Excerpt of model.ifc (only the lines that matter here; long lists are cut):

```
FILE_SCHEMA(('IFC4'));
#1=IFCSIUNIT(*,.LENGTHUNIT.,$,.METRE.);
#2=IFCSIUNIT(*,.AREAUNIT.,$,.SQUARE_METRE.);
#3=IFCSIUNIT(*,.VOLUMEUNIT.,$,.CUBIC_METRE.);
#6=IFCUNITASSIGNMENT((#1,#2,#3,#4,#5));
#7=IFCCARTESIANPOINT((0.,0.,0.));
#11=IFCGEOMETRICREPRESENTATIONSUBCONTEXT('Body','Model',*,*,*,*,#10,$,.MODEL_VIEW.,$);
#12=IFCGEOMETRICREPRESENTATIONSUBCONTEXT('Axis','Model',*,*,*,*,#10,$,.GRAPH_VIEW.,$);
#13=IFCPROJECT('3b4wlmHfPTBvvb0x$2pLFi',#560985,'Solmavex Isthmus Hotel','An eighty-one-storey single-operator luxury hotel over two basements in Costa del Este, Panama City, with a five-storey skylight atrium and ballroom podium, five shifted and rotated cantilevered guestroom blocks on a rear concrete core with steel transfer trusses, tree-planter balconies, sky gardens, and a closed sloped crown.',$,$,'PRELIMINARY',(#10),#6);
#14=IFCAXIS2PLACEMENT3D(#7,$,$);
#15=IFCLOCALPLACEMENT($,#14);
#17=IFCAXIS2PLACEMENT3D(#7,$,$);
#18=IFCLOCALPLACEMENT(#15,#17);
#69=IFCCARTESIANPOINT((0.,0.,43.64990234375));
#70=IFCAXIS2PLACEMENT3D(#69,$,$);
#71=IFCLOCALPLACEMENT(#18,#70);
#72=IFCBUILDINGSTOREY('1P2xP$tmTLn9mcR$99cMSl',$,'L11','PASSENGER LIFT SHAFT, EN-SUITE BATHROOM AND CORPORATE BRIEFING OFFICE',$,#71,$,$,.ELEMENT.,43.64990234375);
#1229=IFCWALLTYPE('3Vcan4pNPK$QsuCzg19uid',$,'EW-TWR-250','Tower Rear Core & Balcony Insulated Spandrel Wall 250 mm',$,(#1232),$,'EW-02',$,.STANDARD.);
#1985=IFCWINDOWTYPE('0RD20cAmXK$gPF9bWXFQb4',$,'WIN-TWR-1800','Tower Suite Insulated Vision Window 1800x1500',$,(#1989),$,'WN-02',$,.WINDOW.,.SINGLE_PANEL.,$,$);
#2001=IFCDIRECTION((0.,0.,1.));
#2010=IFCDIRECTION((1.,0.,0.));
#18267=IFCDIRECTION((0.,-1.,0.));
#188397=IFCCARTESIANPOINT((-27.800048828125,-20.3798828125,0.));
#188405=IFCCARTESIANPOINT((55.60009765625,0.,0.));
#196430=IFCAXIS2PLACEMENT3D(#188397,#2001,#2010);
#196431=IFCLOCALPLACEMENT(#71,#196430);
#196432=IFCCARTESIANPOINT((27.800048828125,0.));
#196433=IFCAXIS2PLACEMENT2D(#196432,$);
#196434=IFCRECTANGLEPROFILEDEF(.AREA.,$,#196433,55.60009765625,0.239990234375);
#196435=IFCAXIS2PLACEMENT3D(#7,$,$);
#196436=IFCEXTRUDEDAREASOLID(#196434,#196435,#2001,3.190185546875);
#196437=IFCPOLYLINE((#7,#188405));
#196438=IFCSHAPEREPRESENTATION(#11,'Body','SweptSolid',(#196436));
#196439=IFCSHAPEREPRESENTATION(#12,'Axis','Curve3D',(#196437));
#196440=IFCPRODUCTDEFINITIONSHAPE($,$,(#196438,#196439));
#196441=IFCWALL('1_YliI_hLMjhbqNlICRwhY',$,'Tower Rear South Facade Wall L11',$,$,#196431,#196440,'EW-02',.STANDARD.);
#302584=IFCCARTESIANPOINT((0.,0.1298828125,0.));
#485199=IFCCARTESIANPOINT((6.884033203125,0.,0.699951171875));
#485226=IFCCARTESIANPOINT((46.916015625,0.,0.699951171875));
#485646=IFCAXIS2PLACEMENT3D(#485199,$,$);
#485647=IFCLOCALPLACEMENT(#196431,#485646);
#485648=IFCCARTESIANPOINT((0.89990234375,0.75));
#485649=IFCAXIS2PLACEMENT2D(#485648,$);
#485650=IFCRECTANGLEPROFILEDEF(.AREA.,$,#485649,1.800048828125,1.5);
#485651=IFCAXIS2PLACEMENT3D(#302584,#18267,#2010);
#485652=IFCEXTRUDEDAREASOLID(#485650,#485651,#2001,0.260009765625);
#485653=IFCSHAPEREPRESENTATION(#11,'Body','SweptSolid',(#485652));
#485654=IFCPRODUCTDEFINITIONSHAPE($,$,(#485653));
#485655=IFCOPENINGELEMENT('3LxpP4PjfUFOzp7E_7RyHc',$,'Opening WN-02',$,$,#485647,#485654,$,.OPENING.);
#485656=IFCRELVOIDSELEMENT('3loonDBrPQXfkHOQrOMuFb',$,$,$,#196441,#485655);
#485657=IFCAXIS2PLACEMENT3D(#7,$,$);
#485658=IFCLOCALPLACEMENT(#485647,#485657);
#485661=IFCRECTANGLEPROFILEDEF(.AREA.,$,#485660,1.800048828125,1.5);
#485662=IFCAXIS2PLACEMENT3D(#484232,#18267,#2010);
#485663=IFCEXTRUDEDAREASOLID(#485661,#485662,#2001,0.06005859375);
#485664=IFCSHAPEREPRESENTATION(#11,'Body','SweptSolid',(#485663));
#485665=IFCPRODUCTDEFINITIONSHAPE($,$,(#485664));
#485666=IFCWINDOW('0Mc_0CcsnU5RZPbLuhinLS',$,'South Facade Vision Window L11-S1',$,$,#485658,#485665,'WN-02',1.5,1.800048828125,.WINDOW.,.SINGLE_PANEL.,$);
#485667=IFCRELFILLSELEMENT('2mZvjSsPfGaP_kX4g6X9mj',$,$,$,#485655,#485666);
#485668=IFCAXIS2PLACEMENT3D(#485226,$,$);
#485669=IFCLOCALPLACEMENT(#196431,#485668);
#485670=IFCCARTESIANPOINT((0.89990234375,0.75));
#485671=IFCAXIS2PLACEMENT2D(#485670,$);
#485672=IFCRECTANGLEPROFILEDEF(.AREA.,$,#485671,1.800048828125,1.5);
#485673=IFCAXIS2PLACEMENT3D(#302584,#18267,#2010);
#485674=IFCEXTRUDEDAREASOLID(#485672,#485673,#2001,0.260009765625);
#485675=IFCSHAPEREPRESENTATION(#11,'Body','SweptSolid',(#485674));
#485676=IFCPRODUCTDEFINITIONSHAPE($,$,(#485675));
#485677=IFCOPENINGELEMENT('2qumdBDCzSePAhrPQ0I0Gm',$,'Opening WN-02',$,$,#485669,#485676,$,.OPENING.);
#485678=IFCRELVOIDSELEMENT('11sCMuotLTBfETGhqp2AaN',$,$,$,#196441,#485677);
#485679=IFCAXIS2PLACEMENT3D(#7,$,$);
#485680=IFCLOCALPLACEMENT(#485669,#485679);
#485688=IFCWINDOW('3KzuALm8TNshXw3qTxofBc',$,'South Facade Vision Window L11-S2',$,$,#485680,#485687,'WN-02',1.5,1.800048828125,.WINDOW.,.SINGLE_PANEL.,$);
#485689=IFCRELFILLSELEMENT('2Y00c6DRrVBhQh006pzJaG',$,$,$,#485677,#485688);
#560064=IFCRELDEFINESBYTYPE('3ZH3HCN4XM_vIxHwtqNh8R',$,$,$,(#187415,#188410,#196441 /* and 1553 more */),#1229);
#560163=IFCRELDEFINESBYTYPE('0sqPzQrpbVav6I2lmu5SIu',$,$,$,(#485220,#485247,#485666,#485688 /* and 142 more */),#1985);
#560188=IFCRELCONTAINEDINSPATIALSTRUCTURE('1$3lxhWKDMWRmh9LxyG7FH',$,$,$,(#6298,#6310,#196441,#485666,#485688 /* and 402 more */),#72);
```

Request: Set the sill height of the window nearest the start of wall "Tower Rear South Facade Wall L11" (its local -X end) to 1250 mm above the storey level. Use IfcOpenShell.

```python
import numpy as np
import ifcopenshell
import ifcopenshell.api.geometry
import ifcopenshell.geom
import ifcopenshell.util.element
import ifcopenshell.util.placement
import ifcopenshell.util.shape
import ifcopenshell.util.unit

model = ifcopenshell.open("model.ifc")
unit_scale = ifcopenshell.util.unit.calculate_unit_scale(model)

window = model.by_id(485666)
opening = window.FillsVoids[0].RelatingOpeningElement
storey = ifcopenshell.util.element.get_container(window, ifc_class="IfcBuildingStorey")
level = ifcopenshell.util.placement.get_local_placement(storey.ObjectPlacement)[2, 3]

# The opening's origin need not be at the sill, so measure its lowest point.
shape = ifcopenshell.geom.create_shape(ifcopenshell.geom.settings(), opening)
bottom = ifcopenshell.util.shape.get_shape_bottom_elevation(shape, shape.geometry) / unit_scale
dz = level + 1.25 / unit_scale - bottom

shift = np.array([0.0, 0.0, dz])
# The window is placed relative to its opening, so it follows when the opening moves.
matrix = ifcopenshell.util.placement.get_local_placement(opening.ObjectPlacement)
matrix[:3, 3] += shift
ifcopenshell.api.geometry.edit_object_placement(
    model, product=opening, matrix=matrix, is_si=False, should_transform_children=True
)

print(f"moved by {dz * unit_scale:+.3f} m")

model.write("model_updated.ifc")
```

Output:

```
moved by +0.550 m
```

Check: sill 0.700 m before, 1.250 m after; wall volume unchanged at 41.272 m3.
